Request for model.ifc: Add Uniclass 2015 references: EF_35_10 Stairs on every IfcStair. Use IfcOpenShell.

First a look at what the model holds.

```python
import ifcopenshell

model = ifcopenshell.open("model.ifc")
print(model.schema)
print("classifications:", [c.Name for c in model.by_type("IfcClassification")])
for ifc_class in ("IfcDoor", "IfcRoof", "IfcStair", "IfcWall", "IfcWindow"):
    print(ifc_class, len(model.by_type(ifc_class)))
```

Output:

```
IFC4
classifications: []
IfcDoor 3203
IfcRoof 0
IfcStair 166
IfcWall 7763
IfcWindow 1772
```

```python
import ifcopenshell
import ifcopenshell.api.classification

model = ifcopenshell.open("model.ifc")

system = ifcopenshell.api.classification.add_classification(model, classification="Uniclass 2015")

codes = {
    "IfcStair": ("EF_35_10", "Stairs"),
}
for ifc_class, (code, name) in codes.items():
    products = model.by_type(ifc_class)
    ifcopenshell.api.classification.add_reference(
        model, products=products, classification=system, identification=code, name=name
    )
    print(code, len(products))

model.write("model_rev.ifc")
```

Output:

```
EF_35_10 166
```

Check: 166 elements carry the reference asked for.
